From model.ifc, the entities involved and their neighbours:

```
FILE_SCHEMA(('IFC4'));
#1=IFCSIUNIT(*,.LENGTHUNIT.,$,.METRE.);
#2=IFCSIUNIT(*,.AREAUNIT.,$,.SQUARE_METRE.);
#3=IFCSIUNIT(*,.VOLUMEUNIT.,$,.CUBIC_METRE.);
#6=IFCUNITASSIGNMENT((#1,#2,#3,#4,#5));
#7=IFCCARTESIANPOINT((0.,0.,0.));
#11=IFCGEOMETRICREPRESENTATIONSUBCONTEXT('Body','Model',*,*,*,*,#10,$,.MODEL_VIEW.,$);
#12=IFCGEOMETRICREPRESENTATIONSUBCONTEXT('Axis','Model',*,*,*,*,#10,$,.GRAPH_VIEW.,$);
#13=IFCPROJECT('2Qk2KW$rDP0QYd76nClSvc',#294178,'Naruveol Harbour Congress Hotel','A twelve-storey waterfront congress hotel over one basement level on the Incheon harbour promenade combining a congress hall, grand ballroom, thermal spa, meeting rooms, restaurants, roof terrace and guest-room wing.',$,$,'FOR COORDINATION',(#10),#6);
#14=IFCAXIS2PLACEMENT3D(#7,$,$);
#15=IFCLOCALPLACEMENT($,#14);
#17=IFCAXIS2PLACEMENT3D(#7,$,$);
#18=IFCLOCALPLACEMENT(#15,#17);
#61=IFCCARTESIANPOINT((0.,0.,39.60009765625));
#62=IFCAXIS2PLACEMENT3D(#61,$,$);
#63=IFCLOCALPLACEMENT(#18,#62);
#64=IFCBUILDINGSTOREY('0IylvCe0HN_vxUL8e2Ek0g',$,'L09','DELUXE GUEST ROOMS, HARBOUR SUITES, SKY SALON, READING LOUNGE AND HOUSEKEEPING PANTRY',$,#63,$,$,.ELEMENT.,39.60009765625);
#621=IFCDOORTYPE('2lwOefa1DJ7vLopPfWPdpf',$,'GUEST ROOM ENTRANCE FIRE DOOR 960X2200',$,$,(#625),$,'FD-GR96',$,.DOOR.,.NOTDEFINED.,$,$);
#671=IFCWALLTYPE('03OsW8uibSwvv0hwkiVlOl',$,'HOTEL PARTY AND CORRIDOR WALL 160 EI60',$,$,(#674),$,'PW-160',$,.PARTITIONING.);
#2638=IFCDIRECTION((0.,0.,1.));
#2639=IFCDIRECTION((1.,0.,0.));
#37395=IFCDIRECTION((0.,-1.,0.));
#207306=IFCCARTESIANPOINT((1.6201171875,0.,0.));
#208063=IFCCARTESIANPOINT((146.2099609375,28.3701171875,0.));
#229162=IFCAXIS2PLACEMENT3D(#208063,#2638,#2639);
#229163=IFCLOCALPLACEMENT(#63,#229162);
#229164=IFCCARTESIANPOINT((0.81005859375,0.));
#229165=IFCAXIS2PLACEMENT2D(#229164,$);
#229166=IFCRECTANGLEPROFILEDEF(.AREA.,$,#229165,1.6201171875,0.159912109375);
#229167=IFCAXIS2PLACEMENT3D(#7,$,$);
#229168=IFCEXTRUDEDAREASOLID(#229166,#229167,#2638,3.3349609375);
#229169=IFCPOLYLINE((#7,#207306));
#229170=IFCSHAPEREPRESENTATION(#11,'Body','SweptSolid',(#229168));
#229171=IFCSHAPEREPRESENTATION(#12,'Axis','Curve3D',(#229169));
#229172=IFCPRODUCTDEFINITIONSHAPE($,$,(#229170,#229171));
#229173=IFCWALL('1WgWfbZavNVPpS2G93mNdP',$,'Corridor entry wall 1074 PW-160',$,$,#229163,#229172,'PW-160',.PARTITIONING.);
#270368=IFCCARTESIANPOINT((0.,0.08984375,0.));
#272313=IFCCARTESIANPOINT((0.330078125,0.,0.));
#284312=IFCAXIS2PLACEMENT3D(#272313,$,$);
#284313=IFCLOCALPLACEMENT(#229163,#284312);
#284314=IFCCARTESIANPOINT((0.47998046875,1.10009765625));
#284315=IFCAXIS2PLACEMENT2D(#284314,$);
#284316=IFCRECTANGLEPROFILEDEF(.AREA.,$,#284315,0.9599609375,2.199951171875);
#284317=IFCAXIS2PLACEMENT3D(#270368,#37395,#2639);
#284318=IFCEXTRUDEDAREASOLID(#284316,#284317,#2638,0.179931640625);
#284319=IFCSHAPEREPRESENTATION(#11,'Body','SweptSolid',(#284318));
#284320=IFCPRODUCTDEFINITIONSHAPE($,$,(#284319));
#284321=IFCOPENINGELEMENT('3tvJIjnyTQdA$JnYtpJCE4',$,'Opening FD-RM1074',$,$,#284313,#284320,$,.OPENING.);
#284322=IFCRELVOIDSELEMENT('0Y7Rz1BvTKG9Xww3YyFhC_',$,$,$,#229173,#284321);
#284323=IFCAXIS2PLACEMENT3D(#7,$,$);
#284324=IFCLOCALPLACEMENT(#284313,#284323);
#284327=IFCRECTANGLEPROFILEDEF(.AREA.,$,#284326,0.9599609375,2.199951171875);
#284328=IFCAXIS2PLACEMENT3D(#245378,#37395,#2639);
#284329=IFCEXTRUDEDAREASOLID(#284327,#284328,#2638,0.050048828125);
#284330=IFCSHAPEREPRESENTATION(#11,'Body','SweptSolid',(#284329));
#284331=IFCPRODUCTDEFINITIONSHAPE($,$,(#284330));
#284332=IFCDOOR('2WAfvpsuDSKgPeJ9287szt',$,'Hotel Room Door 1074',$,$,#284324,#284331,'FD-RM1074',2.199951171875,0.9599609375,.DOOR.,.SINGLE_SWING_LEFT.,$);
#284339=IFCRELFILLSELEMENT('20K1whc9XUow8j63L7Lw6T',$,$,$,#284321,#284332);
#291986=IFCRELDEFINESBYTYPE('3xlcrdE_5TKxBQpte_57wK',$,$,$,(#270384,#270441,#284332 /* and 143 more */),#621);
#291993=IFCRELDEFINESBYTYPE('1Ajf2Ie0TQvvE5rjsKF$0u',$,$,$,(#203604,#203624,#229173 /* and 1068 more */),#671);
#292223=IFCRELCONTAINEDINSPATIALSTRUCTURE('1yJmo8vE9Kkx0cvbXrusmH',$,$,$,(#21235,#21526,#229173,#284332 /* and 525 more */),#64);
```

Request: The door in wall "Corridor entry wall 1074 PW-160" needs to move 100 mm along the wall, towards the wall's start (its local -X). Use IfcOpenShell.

```python
import ifcopenshell
import ifcopenshell.api.geometry
import ifcopenshell.util.placement

model = ifcopenshell.open("model.ifc")

door = model.by_guid("2WAfvpsuDSKgPeJ9287szt")
opening = door.FillsVoids[0].RelatingOpeningElement
wall = opening.VoidsElements[0].RelatingBuildingElement

wall_matrix = ifcopenshell.util.placement.get_local_placement(wall.ObjectPlacement)
shift = wall_matrix[:3, 0] * -0.1
before = ifcopenshell.util.placement.get_local_placement(door.ObjectPlacement)[:3, 3].copy()

# The door is placed relative to its opening, so it follows when the opening moves.
matrix = ifcopenshell.util.placement.get_local_placement(opening.ObjectPlacement)
matrix[:3, 3] += shift
ifcopenshell.api.geometry.edit_object_placement(
    model, product=opening, matrix=matrix, is_si=False, should_transform_children=True
)

after = ifcopenshell.util.placement.get_local_placement(door.ObjectPlacement)[:3, 3]
print("door moved by", (after - before).round(3) + 0.0)

model.write("model_v2.ifc")
```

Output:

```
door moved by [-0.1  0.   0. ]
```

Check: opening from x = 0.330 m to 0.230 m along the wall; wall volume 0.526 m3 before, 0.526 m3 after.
